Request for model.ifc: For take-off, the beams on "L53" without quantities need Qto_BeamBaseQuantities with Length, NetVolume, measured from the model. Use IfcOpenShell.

First a look at what the model holds.

```python
import ifcopenshell
import ifcopenshell.util.element
import ifcopenshell.util.unit

model = ifcopenshell.open("model.ifc")
print(model.schema)
for unit_type in ("LENGTHUNIT", "AREAUNIT", "VOLUMEUNIT"):
    print(unit_type, ifcopenshell.util.unit.calculate_unit_scale(model, unit_type))
storey = next(s for s in model.by_type("IfcBuildingStorey") if s.Name == "L53")
beams = [e for e in ifcopenshell.util.element.get_decomposition(storey) if e.is_a("IfcBeam")]
for e in sorted(beams, key=lambda e: e.id()):
    print(e.id(), e.is_a(), e.Name, list(ifcopenshell.util.element.get_psets(e, qtos_only=True)), sep=" | ")
```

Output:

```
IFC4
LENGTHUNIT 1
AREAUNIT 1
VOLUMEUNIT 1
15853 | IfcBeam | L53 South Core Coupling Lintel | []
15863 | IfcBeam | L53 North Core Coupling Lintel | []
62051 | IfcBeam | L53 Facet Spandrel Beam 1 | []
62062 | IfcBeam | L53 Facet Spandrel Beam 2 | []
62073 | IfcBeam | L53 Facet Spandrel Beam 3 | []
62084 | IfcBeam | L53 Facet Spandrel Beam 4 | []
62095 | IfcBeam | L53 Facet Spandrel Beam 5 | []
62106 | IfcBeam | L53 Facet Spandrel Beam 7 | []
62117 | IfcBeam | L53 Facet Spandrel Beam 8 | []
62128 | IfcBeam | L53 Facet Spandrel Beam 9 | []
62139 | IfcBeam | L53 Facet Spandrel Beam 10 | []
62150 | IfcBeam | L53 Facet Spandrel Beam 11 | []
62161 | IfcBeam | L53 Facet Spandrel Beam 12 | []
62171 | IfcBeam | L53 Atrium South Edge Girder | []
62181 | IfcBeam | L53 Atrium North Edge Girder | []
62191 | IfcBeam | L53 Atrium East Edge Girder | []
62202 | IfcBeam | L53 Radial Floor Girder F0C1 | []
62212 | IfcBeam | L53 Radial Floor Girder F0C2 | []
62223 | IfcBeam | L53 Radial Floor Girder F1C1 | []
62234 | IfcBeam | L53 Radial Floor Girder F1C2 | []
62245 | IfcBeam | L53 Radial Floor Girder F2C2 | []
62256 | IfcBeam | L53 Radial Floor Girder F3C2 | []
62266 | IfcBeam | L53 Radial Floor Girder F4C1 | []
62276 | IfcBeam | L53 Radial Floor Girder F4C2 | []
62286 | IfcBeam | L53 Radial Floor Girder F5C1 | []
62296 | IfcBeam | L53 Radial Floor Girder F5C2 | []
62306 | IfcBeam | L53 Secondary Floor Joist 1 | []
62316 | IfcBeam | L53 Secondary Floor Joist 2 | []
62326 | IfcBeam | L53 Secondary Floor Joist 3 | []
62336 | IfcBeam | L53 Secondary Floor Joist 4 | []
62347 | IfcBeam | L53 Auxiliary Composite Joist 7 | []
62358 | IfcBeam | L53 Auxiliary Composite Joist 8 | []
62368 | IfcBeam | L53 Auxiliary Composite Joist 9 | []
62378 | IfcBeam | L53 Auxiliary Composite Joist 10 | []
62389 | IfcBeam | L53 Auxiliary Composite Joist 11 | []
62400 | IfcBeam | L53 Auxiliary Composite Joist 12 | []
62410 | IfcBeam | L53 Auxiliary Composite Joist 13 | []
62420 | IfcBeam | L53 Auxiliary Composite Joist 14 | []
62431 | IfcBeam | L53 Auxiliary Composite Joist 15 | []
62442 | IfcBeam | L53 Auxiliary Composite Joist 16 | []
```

```python
import ifcopenshell
import ifcopenshell.api.pset
import ifcopenshell.geom
import ifcopenshell.util.element
import ifcopenshell.util.shape
import ifcopenshell.util.unit

model = ifcopenshell.open("model.ifc")
unit_scale = ifcopenshell.util.unit.calculate_unit_scale(model)
volume_scale = ifcopenshell.util.unit.calculate_unit_scale(model, "VOLUMEUNIT")
settings = ifcopenshell.geom.settings()

storey = next(s for s in model.by_type("IfcBuildingStorey") if s.Name == "L53")
beams = [e for e in ifcopenshell.util.element.get_decomposition(storey) if e.is_a("IfcBeam")]

for e in sorted(beams, key=lambda e: e.id()):
    if ifcopenshell.util.element.get_psets(e, qtos_only=True, should_inherit=False):
        continue
    # Geometry comes back in metres, in the element's own axes.
    shape = ifcopenshell.geom.create_shape(settings, e)
    values = {
        "Length": ifcopenshell.util.shape.get_max_xyz(shape.geometry) / unit_scale,
        "NetVolume": ifcopenshell.util.shape.get_volume(shape.geometry) / volume_scale,
    }
    qto = ifcopenshell.api.pset.add_qto(model, product=e, name="Qto_BeamBaseQuantities")
    ifcopenshell.api.pset.edit_qto(model, qto=qto, properties=values)
    print(e.id(), {k: round(v, 3) for k, v in values.items()})

model.write("model_edited.ifc")
```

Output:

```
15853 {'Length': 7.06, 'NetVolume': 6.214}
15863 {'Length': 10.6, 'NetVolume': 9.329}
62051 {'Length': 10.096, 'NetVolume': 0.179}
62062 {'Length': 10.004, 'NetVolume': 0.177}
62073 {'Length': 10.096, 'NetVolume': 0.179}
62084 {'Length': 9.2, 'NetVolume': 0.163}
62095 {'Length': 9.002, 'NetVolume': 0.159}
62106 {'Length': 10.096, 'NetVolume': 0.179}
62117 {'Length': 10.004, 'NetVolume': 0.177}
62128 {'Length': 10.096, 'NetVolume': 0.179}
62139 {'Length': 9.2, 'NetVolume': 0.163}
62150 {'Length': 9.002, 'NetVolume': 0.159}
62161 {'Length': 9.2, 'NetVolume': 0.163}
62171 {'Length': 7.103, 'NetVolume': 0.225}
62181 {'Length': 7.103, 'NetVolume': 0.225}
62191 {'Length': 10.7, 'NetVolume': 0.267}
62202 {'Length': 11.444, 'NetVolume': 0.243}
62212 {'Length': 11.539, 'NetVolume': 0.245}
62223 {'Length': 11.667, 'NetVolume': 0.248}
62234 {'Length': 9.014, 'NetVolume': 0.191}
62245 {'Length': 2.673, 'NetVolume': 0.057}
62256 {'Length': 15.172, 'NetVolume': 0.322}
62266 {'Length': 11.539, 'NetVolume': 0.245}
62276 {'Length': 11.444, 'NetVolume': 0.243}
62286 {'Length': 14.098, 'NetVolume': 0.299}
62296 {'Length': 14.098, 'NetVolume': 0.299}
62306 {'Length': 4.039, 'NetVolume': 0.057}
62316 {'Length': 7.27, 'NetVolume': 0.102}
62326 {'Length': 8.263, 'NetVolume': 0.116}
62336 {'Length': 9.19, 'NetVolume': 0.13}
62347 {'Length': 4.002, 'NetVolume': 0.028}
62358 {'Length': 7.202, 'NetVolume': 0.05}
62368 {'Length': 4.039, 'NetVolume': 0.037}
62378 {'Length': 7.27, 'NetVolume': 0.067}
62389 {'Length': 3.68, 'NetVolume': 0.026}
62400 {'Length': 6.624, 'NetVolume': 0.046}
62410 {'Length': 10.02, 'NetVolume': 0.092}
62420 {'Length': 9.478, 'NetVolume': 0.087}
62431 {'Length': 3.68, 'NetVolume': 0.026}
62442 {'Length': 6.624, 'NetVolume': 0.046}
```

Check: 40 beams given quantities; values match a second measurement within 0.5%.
